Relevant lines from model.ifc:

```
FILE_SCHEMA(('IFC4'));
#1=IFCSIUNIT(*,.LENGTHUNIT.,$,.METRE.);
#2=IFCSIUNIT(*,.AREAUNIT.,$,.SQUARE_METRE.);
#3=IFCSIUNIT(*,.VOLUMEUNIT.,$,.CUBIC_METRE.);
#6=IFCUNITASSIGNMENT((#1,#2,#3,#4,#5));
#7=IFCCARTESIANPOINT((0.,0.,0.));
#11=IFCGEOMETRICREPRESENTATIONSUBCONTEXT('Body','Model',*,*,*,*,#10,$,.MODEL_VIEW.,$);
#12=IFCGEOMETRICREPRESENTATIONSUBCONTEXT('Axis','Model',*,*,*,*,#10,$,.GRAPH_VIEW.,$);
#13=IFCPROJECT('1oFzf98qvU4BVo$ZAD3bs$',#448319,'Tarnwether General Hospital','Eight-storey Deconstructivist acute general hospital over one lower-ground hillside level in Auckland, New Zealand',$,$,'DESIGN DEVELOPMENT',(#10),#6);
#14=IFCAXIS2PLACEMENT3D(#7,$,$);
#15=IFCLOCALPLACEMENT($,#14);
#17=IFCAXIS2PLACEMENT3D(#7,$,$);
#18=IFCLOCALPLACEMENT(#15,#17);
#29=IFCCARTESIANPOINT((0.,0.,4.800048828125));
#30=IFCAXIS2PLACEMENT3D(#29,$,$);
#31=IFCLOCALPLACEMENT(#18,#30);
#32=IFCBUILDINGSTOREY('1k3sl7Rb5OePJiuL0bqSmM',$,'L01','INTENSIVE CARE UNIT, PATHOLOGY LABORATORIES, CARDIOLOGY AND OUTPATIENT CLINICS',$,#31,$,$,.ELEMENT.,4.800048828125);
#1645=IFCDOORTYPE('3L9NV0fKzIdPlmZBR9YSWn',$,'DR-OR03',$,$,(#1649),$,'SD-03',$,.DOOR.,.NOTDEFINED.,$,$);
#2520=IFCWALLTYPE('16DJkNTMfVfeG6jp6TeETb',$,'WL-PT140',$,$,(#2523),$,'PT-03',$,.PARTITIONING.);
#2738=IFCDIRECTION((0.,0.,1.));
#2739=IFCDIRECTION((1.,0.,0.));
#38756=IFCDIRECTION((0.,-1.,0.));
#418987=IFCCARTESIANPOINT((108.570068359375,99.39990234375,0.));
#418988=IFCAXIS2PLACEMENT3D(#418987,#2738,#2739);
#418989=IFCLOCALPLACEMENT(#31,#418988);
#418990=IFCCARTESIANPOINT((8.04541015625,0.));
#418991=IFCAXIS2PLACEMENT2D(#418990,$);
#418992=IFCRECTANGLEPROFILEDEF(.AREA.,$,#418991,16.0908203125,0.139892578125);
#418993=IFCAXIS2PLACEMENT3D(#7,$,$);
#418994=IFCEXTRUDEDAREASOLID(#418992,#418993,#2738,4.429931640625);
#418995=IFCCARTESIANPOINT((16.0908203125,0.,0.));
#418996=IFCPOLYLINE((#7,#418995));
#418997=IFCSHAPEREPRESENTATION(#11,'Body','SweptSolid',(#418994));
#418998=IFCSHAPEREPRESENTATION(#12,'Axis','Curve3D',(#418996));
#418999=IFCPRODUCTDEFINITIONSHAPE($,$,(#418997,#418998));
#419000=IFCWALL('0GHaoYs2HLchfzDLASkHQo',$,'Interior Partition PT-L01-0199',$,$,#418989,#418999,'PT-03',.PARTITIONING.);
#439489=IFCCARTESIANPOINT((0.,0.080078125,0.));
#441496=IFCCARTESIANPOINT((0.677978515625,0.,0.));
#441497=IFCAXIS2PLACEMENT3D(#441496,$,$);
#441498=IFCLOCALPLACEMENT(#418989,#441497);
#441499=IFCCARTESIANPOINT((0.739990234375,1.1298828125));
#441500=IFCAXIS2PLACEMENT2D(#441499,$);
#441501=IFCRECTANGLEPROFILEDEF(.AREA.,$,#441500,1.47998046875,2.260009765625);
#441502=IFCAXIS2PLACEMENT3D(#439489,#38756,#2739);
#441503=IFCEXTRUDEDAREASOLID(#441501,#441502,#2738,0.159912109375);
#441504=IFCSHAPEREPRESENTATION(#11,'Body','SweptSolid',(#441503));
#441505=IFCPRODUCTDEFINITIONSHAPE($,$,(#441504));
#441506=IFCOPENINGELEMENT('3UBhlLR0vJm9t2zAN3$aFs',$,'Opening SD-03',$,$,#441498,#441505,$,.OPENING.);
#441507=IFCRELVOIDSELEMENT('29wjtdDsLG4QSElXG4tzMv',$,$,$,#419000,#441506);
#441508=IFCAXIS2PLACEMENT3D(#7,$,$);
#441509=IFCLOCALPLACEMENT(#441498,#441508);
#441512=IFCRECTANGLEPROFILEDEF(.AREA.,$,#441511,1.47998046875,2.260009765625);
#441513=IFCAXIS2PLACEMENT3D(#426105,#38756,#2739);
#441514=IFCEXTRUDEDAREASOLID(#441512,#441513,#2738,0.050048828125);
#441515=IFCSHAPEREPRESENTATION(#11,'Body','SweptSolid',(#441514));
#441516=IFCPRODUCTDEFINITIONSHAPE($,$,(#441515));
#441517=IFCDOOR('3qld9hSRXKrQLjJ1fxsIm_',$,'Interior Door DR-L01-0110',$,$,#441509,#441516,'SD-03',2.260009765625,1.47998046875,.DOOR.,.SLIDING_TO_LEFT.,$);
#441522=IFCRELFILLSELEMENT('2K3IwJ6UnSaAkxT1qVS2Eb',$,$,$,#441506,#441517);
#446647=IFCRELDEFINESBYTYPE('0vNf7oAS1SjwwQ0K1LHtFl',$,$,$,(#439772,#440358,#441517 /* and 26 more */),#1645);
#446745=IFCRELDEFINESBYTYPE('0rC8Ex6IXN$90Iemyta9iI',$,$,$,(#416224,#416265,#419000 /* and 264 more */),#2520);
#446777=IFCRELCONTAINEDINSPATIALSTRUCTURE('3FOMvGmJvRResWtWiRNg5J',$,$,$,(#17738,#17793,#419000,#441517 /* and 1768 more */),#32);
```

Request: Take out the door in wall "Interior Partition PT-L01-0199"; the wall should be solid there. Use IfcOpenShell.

```python
import ifcopenshell
import ifcopenshell.api.feature
import ifcopenshell.api.root
import ifcopenshell.geom
import ifcopenshell.util.shape

model = ifcopenshell.open("model.ifc")
settings = ifcopenshell.geom.settings()


def volume(element):
    """Net volume in cubic metres, openings subtracted."""
    shape = ifcopenshell.geom.create_shape(settings, element)
    return ifcopenshell.util.shape.get_volume(shape.geometry)


door = model.by_guid("3qld9hSRXKrQLjJ1fxsIm_")
opening = door.FillsVoids[0].RelatingOpeningElement
wall = opening.VoidsElements[0].RelatingBuildingElement
before = volume(wall)

ifcopenshell.api.root.remove_product(model, product=door)
ifcopenshell.api.feature.remove_feature(model, feature=opening)

after = volume(wall)

print(f"wall volume {before:.3f} -> {after:.3f} m3")

model.write("model_edited.ifc")
```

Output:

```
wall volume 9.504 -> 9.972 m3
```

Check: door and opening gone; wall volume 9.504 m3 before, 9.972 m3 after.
